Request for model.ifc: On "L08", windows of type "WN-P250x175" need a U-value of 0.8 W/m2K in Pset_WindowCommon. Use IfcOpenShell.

First a look at what the model holds.

```python
import ifcopenshell
import ifcopenshell.util.element

model = ifcopenshell.open("model.ifc")
print(model.schema)
storey = next(s for s in model.by_type("IfcBuildingStorey") if s.Name == "L08")
windows = [e for e in ifcopenshell.util.element.get_decomposition(storey) if e.is_a("IfcWindow")]
seen = {}
for e in windows:
    element_type = ifcopenshell.util.element.get_type(e)
    key = (element_type.Name if element_type != e and element_type else None, ifcopenshell.util.element.get_pset(e, "Pset_WindowCommon", "ThermalTransmittance"))
    seen[key] = seen.get(key, 0) + 1
for (name, value), count in sorted(seen.items(), key=str):
    print(count, "x", name, "|", value)
```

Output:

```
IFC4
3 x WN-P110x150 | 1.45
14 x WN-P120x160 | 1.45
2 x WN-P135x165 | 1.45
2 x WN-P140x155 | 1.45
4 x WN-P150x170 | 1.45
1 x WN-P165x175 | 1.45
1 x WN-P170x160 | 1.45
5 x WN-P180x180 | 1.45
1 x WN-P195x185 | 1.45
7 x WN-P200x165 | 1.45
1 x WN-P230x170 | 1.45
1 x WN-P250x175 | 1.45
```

```python
import ifcopenshell
import ifcopenshell.api.pset
import ifcopenshell.util.element

model = ifcopenshell.open("model.ifc")

storey = next(s for s in model.by_type("IfcBuildingStorey") if s.Name == "L08")
windows = [e for e in ifcopenshell.util.element.get_decomposition(storey) if e.is_a("IfcWindow")]

count = 0
for e in windows:
    element_type = ifcopenshell.util.element.get_type(e)
    if element_type in (None, e) or element_type.Name != "WN-P250x175":
        continue
    # add_pset returns the element's existing set when there is one.
    pset = ifcopenshell.api.pset.add_pset(model, product=e, name="Pset_WindowCommon")
    ifcopenshell.api.pset.edit_pset(model, pset=pset, properties={"ThermalTransmittance": 0.8})
    count += 1

print(count, "windows updated")

model.write("model_rev.ifc")
```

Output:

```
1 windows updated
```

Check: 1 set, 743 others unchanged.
